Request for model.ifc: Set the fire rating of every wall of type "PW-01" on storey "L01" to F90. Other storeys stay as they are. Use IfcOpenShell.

First a look at what the model holds.

```python
import ifcopenshell
import ifcopenshell.util.element

model = ifcopenshell.open("model.ifc")
print(model.schema)
storey = next(s for s in model.by_type("IfcBuildingStorey") if s.Name == "L01")
walls = [e for e in ifcopenshell.util.element.get_decomposition(storey) if e.is_a("IfcWall")]
seen = {}
for e in walls:
    element_type = ifcopenshell.util.element.get_type(e)
    key = (element_type.Name if element_type != e and element_type else None, ifcopenshell.util.element.get_pset(e, "Pset_WallCommon", "FireRating"))
    seen[key] = seen.get(key, 0) + 1
for (name, value), count in sorted(seen.items(), key=str):
    print(count, "x", name, "|", value)
```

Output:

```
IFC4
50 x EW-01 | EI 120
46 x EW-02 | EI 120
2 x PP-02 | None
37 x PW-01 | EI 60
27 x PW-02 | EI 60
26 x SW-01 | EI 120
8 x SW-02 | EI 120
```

```python
import ifcopenshell
import ifcopenshell.api.pset
import ifcopenshell.util.element

model = ifcopenshell.open("model.ifc")

storey = next(s for s in model.by_type("IfcBuildingStorey") if s.Name == "L01")
walls = [e for e in ifcopenshell.util.element.get_decomposition(storey) if e.is_a("IfcWall")]

count = 0
for e in walls:
    element_type = ifcopenshell.util.element.get_type(e)
    if element_type in (None, e) or element_type.Name != "PW-01":
        continue
    # add_pset returns the element's existing set when there is one.
    pset = ifcopenshell.api.pset.add_pset(model, product=e, name="Pset_WallCommon")
    ifcopenshell.api.pset.edit_pset(model, pset=pset, properties={"FireRating": "F90"})
    count += 1

print(count, "walls updated")

model.write("model_v2.ifc")
```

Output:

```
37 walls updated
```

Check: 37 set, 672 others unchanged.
